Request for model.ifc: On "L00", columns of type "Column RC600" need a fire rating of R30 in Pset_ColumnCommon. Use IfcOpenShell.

First a look at what the model holds.

```python
import ifcopenshell
import ifcopenshell.util.element

model = ifcopenshell.open("model.ifc")
print(model.schema)
storey = next(s for s in model.by_type("IfcBuildingStorey") if s.Name == "L00")
columns = [e for e in ifcopenshell.util.element.get_decomposition(storey) if e.is_a("IfcColumn")]
seen = {}
for e in columns:
    element_type = ifcopenshell.util.element.get_type(e)
    key = (element_type.Name if element_type != e and element_type else None, ifcopenshell.util.element.get_pset(e, "Pset_ColumnCommon", "FireRating"))
    seen[key] = seen.get(key, 0) + 1
for (name, value), count in sorted(seen.items(), key=str):
    print(count, "x", name, "|", value)
```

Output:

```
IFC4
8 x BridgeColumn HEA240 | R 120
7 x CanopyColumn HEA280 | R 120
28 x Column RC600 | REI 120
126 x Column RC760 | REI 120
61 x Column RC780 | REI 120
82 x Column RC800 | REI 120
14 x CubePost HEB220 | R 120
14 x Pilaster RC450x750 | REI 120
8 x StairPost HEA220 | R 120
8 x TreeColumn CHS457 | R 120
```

```python
import ifcopenshell
import ifcopenshell.api.pset
import ifcopenshell.util.element

model = ifcopenshell.open("model.ifc")

storey = next(s for s in model.by_type("IfcBuildingStorey") if s.Name == "L00")
columns = [e for e in ifcopenshell.util.element.get_decomposition(storey) if e.is_a("IfcColumn")]

count = 0
for e in columns:
    element_type = ifcopenshell.util.element.get_type(e)
    if element_type in (None, e) or element_type.Name != "Column RC600":
        continue
    # add_pset returns the element's existing set when there is one.
    pset = ifcopenshell.api.pset.add_pset(model, product=e, name="Pset_ColumnCommon")
    ifcopenshell.api.pset.edit_pset(model, pset=pset, properties={"FireRating": "R30"})
    count += 1

print(count, "columns updated")

model.write("model-out.ifc")
```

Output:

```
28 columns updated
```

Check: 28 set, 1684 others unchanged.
